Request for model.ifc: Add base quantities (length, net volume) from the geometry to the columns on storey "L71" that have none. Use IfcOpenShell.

First a look at what the model holds.

```python
import ifcopenshell
import ifcopenshell.util.element
import ifcopenshell.util.unit

model = ifcopenshell.open("model.ifc")
print(model.schema)
for unit_type in ("LENGTHUNIT", "AREAUNIT", "VOLUMEUNIT"):
    print(unit_type, ifcopenshell.util.unit.calculate_unit_scale(model, unit_type))
storey = next(s for s in model.by_type("IfcBuildingStorey") if s.Name == "L71")
columns = [e for e in ifcopenshell.util.element.get_decomposition(storey) if e.is_a("IfcColumn")]
for e in sorted(columns, key=lambda e: e.id()):
    print(e.id(), e.is_a(), e.Name, list(ifcopenshell.util.element.get_psets(e, qtos_only=True)), sep=" | ")
```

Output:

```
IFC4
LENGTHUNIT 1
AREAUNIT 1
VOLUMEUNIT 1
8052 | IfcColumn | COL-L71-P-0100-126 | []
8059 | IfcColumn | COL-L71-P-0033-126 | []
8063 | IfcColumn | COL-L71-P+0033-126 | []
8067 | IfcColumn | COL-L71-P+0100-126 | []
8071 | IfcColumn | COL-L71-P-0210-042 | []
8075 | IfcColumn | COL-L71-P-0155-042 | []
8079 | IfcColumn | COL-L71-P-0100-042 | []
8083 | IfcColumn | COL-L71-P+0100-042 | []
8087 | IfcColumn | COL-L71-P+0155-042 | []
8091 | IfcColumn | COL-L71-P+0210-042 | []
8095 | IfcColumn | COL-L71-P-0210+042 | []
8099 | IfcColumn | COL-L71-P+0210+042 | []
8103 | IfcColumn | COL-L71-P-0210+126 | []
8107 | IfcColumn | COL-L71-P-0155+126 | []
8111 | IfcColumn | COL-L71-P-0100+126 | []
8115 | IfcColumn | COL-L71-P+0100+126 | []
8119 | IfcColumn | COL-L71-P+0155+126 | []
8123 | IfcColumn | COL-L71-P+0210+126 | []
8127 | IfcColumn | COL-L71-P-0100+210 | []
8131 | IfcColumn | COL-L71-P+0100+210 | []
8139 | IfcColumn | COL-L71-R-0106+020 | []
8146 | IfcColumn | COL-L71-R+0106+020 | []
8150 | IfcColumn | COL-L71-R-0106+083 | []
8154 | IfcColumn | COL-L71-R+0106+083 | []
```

```python
import ifcopenshell
import ifcopenshell.api.pset
import ifcopenshell.geom
import ifcopenshell.util.element
import ifcopenshell.util.shape
import ifcopenshell.util.unit

model = ifcopenshell.open("model.ifc")
unit_scale = ifcopenshell.util.unit.calculate_unit_scale(model)
volume_scale = ifcopenshell.util.unit.calculate_unit_scale(model, "VOLUMEUNIT")
settings = ifcopenshell.geom.settings()

storey = next(s for s in model.by_type("IfcBuildingStorey") if s.Name == "L71")
columns = [e for e in ifcopenshell.util.element.get_decomposition(storey) if e.is_a("IfcColumn")]

for e in sorted(columns, key=lambda e: e.id()):
    if ifcopenshell.util.element.get_psets(e, qtos_only=True, should_inherit=False):
        continue
    # Geometry comes back in metres, in the element's own axes.
    shape = ifcopenshell.geom.create_shape(settings, e)
    values = {
        "Length": ifcopenshell.util.shape.get_z(shape.geometry) / unit_scale,
        "NetVolume": ifcopenshell.util.shape.get_volume(shape.geometry) / volume_scale,
    }
    qto = ifcopenshell.api.pset.add_qto(model, product=e, name="Qto_ColumnBaseQuantities")
    ifcopenshell.api.pset.edit_qto(model, qto=qto, properties=values)
    print(e.id(), {k: round(v, 3) for k, v in values.items()})

model.write("model-out.ifc")
```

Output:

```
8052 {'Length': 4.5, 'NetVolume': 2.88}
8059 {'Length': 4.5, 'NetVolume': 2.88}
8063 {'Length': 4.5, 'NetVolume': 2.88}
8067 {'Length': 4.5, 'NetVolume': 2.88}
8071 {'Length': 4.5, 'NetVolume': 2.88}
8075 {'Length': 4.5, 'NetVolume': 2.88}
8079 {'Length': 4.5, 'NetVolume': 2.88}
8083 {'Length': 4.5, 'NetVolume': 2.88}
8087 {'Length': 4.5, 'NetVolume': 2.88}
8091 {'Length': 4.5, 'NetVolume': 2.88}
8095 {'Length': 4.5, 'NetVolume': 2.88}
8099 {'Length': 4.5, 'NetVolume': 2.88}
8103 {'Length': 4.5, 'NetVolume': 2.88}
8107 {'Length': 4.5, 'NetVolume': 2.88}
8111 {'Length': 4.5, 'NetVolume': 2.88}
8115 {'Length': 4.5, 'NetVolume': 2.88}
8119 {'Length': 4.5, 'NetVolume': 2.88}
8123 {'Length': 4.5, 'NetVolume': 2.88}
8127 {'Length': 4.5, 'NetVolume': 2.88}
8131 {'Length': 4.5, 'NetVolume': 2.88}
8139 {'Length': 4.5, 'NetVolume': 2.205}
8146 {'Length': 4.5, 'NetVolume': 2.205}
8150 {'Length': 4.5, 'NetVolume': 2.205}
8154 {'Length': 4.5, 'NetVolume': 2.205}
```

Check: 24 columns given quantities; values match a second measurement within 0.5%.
